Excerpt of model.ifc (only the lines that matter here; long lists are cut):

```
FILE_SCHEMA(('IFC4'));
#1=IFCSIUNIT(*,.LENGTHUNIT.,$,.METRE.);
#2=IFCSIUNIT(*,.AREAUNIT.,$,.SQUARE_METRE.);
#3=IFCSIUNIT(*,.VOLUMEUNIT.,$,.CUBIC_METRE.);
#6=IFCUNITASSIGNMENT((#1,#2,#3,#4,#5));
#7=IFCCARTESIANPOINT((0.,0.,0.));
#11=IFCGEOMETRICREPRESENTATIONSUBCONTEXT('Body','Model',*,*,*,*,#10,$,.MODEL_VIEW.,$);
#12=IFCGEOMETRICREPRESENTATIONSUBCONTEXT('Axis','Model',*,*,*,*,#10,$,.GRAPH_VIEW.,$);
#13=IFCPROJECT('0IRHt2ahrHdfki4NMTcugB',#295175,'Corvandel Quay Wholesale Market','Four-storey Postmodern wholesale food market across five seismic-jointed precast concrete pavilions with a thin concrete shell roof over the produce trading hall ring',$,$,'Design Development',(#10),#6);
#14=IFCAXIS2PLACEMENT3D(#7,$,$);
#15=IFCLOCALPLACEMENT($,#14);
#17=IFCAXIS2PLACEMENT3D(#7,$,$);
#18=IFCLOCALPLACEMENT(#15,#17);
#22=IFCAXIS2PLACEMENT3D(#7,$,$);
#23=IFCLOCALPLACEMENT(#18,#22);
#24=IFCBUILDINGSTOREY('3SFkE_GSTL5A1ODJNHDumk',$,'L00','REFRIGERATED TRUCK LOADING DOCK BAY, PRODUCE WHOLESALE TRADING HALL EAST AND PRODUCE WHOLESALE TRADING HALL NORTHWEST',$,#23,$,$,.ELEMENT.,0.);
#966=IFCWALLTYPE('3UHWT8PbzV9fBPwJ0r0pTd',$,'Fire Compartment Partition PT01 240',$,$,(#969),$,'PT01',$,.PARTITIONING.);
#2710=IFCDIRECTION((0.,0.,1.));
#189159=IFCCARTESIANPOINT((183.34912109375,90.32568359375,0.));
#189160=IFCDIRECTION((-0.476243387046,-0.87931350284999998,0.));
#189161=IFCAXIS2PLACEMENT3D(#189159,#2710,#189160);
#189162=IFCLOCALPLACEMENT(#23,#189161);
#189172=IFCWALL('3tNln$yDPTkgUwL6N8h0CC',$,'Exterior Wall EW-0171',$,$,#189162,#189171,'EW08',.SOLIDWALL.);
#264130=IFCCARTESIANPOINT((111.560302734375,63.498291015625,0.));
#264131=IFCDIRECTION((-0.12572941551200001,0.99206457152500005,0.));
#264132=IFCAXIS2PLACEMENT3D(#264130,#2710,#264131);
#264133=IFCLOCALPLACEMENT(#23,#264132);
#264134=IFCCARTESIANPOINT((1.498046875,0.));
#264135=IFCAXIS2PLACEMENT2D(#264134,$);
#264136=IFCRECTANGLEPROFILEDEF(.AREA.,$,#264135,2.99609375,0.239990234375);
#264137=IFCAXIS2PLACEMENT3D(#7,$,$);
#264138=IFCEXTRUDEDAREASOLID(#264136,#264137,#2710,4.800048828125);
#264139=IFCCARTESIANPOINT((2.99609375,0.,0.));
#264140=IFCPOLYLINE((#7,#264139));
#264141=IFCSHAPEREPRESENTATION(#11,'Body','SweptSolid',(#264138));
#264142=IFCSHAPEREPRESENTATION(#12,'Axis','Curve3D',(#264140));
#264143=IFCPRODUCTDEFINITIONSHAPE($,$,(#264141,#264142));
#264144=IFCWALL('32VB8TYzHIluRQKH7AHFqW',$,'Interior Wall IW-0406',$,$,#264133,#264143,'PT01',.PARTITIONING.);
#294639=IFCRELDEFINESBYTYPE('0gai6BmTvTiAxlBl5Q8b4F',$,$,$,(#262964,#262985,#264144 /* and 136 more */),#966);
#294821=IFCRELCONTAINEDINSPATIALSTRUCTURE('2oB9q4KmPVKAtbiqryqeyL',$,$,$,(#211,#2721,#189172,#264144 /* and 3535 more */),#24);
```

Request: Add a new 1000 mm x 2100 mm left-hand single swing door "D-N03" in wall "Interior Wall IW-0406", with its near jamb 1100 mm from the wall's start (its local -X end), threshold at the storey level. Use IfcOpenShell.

```python
import numpy as np
import ifcopenshell
import ifcopenshell.api.feature
import ifcopenshell.api.geometry
import ifcopenshell.api.root
import ifcopenshell.api.spatial
import ifcopenshell.geom
import ifcopenshell.util.element
import ifcopenshell.util.placement
import ifcopenshell.util.representation
import ifcopenshell.util.shape
import ifcopenshell.util.unit

model = ifcopenshell.open("model.ifc")
unit_scale = ifcopenshell.util.unit.calculate_unit_scale(model)
settings = ifcopenshell.geom.settings()


def volume(element):
    """Net volume in cubic metres, openings subtracted."""
    shape = ifcopenshell.geom.create_shape(settings, element)
    return ifcopenshell.util.shape.get_volume(shape.geometry)


wall = model.by_guid("32VB8TYzHIluRQKH7AHFqW")
storey = ifcopenshell.util.element.get_container(wall, ifc_class="IfcBuildingStorey")
context = ifcopenshell.util.representation.get_context(model, "Model", "Body", "MODEL_VIEW")
before = volume(wall)

width, height, from_end, sill = 1, 2.1, 1.1, 0.0  # metres

# The wall runs along its own X axis, and the end named is its -X end.
wall_shape = ifcopenshell.geom.create_shape(settings, wall)
x, y, z = ifcopenshell.util.shape.get_vertices(wall_shape.geometry).T
start = x.min() + from_end
face, thickness = float(y.min()), float(y.max() - y.min())
wall_matrix = ifcopenshell.util.placement.get_local_placement(wall.ObjectPlacement)
level = ifcopenshell.util.placement.get_local_placement(storey.ObjectPlacement)[2, 3]


def in_wall(x, y):
    """Placement at x, y metres in the wall's axes, at sill height."""
    matrix = wall_matrix.copy()
    matrix[:, 3] = wall_matrix @ np.array([x / unit_scale, y / unit_scale, 0.0, 1.0])
    matrix[2, 3] = level + sill / unit_scale
    return matrix


# Opening: a box that overshoots both wall faces by 50 mm.
opening = ifcopenshell.api.root.create_entity(model, ifc_class="IfcOpeningElement", predefined_type="OPENING")
box = ifcopenshell.api.geometry.add_wall_representation(
    model, context=context, length=width, height=height, thickness=thickness + 0.1
)
ifcopenshell.api.geometry.assign_representation(model, product=opening, representation=box)
ifcopenshell.api.geometry.edit_object_placement(model, product=opening, matrix=in_wall(start, face - 0.05), is_si=False)
ifcopenshell.api.feature.add_feature(model, feature=opening, element=wall)

door = ifcopenshell.api.root.create_entity(model, ifc_class="IfcDoor", name="D-N03", predefined_type="DOOR")
door.OverallWidth, door.OverallHeight = width / unit_scale, height / unit_scale
door.OperationType = "SINGLE_SWING_LEFT"
body = ifcopenshell.api.geometry.add_door_representation(
    model,
    context=context,
    overall_width=door.OverallWidth,
    overall_height=door.OverallHeight,
    operation_type="SINGLE_SWING_LEFT",
    lining_properties={"LiningDepth": thickness / unit_scale, "ThresholdDepth": thickness / unit_scale},
)
ifcopenshell.api.geometry.assign_representation(model, product=door, representation=body)
ifcopenshell.api.spatial.assign_container(model, products=[door], relating_structure=storey)
ifcopenshell.api.feature.add_filling(model, opening=opening, element=door)

# The lining spans the wall, so the door starts at the wall face.
ifcopenshell.api.geometry.edit_object_placement(model, product=door, matrix=in_wall(start, face), is_si=False)

after = volume(wall)

print(f"wall volume {before:.3f} -> {after:.3f} m3")

model.write("model_v2.ifc")
```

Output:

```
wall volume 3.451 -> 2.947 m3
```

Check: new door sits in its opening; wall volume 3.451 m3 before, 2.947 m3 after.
